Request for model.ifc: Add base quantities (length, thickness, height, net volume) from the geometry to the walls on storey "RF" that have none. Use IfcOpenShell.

First a look at what the model holds.

```python
import ifcopenshell
import ifcopenshell.util.element
import ifcopenshell.util.unit

model = ifcopenshell.open("model.ifc")
print(model.schema)
for unit_type in ("LENGTHUNIT", "AREAUNIT", "VOLUMEUNIT"):
    print(unit_type, ifcopenshell.util.unit.calculate_unit_scale(model, unit_type))
storey = next(s for s in model.by_type("IfcBuildingStorey") if s.Name == "RF")
walls = [e for e in ifcopenshell.util.element.get_decomposition(storey) if e.is_a("IfcWall")]
for e in sorted(walls, key=lambda e: e.id()):
    print(e.id(), e.is_a(), e.Name, list(ifcopenshell.util.element.get_psets(e, qtos_only=True)), sep=" | ")
```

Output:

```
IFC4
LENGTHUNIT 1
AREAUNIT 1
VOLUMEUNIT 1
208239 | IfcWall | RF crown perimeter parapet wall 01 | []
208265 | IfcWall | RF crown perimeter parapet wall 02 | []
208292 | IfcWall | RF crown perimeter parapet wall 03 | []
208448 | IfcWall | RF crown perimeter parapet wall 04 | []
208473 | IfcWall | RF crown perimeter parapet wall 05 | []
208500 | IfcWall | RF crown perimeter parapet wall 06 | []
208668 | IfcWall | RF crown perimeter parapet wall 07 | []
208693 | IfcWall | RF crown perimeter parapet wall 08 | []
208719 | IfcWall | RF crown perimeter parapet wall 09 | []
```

```python
import ifcopenshell
import ifcopenshell.api.pset
import ifcopenshell.geom
import ifcopenshell.util.element
import ifcopenshell.util.shape
import ifcopenshell.util.unit

model = ifcopenshell.open("model.ifc")
unit_scale = ifcopenshell.util.unit.calculate_unit_scale(model)
volume_scale = ifcopenshell.util.unit.calculate_unit_scale(model, "VOLUMEUNIT")
settings = ifcopenshell.geom.settings()

storey = next(s for s in model.by_type("IfcBuildingStorey") if s.Name == "RF")
walls = [e for e in ifcopenshell.util.element.get_decomposition(storey) if e.is_a("IfcWall")]

for e in sorted(walls, key=lambda e: e.id()):
    if ifcopenshell.util.element.get_psets(e, qtos_only=True, should_inherit=False):
        continue
    # Geometry comes back in metres, in the element's own axes.
    shape = ifcopenshell.geom.create_shape(settings, e)
    values = {
        "Length": ifcopenshell.util.shape.get_x(shape.geometry) / unit_scale,
        "Width": ifcopenshell.util.shape.get_y(shape.geometry) / unit_scale,
        "Height": ifcopenshell.util.shape.get_z(shape.geometry) / unit_scale,
        "NetVolume": ifcopenshell.util.shape.get_volume(shape.geometry) / volume_scale,
    }
    qto = ifcopenshell.api.pset.add_qto(model, product=e, name="Qto_WallBaseQuantities")
    ifcopenshell.api.pset.edit_qto(model, qto=qto, properties=values)
    print(e.id(), {k: round(v, 3) for k, v in values.items()})

model.write("model_v2.ifc")
```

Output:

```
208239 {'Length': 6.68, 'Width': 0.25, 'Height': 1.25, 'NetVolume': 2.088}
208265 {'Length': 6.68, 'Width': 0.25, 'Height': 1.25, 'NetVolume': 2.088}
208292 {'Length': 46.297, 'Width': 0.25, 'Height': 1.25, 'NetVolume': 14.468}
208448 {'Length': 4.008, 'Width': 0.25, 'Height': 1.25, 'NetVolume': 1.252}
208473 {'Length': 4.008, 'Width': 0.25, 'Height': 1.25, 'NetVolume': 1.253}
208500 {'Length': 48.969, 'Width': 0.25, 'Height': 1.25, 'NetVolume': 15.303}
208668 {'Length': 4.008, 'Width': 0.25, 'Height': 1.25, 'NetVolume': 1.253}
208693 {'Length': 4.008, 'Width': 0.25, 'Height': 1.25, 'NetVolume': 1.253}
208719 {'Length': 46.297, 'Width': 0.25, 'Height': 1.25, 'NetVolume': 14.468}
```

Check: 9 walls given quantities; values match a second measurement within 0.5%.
